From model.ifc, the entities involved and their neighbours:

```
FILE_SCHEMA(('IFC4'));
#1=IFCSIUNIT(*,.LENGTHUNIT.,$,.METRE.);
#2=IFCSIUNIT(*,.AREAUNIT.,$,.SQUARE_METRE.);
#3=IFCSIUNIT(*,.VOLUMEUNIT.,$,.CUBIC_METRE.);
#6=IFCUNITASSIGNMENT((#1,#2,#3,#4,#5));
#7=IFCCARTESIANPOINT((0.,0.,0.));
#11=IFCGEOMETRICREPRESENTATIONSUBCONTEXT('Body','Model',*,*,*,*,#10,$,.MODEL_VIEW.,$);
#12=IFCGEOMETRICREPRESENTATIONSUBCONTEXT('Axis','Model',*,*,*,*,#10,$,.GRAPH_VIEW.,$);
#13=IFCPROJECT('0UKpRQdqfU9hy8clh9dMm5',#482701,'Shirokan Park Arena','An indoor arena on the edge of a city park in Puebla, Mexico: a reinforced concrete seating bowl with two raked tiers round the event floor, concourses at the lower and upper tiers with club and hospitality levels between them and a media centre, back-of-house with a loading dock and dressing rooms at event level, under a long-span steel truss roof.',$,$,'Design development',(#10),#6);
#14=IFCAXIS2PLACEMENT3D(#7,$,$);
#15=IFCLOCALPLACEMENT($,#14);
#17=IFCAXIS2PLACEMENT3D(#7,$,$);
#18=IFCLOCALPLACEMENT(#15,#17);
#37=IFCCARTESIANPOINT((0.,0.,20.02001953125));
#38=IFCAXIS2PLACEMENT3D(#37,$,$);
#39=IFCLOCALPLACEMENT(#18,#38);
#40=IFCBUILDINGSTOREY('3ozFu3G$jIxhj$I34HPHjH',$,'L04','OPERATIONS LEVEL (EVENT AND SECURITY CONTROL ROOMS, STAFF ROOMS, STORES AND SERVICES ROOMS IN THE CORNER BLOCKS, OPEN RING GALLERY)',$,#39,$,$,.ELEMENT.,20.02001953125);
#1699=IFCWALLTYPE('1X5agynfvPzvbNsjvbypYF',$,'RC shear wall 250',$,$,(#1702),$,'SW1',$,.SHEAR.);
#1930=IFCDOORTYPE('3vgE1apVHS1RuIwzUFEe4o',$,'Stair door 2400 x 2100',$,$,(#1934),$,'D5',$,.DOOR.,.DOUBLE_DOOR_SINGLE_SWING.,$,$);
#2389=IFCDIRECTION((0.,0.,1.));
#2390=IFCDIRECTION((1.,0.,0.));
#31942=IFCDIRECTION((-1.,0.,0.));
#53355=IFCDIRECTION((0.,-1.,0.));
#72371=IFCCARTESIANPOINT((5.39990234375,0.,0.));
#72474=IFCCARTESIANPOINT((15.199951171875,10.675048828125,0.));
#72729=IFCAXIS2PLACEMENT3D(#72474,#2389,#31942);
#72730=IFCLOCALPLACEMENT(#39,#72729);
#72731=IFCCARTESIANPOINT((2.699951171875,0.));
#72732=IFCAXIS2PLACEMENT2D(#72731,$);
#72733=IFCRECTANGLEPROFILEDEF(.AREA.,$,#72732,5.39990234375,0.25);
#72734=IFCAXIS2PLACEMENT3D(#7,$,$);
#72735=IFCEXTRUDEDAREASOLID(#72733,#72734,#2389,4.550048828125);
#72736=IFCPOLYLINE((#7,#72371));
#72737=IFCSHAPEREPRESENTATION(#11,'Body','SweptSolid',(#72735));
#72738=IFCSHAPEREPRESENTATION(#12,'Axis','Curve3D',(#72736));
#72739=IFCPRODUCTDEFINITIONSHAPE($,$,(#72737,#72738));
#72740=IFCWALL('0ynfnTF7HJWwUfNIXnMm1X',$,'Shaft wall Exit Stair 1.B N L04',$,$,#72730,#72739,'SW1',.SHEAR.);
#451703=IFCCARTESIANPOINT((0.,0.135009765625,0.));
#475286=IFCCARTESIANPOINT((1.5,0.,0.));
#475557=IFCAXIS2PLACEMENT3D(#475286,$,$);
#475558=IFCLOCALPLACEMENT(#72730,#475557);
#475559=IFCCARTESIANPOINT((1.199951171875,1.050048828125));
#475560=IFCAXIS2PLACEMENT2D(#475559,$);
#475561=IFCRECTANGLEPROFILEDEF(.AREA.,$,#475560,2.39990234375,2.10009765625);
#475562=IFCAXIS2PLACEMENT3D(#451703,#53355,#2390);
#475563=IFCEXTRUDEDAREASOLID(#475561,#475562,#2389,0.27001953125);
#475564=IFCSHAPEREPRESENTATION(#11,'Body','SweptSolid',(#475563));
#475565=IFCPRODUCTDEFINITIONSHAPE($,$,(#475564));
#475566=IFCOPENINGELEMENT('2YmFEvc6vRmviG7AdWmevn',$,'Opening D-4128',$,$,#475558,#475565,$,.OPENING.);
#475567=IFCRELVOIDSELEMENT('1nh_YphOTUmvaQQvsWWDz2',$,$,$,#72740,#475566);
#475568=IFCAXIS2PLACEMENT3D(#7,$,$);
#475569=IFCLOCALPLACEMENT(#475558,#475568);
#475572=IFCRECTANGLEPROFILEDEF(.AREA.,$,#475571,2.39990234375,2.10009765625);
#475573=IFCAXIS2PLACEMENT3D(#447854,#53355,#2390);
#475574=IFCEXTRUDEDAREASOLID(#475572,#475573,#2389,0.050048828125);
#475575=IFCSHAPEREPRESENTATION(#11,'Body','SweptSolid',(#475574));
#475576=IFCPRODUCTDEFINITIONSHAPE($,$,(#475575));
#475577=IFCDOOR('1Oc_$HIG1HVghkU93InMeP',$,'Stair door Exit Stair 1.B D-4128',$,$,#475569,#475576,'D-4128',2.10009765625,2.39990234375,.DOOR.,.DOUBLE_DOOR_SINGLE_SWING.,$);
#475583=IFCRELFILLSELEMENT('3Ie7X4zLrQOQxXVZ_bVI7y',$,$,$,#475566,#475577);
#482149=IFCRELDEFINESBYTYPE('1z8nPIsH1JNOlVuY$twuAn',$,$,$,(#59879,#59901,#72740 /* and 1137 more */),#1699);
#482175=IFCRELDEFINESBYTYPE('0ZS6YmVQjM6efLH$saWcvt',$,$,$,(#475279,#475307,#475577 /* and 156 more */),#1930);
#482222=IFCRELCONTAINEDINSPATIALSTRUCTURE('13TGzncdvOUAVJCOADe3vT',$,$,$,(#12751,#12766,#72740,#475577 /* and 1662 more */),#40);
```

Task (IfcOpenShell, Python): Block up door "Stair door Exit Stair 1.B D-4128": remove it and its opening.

```python
import ifcopenshell
import ifcopenshell.api.feature
import ifcopenshell.api.root
import ifcopenshell.geom
import ifcopenshell.util.shape

model = ifcopenshell.open("model.ifc")
settings = ifcopenshell.geom.settings()


def volume(element):
    """Net volume in cubic metres, openings subtracted."""
    shape = ifcopenshell.geom.create_shape(settings, element)
    return ifcopenshell.util.shape.get_volume(shape.geometry)


door = model.by_guid("1Oc_$HIG1HVghkU93InMeP")
opening = door.FillsVoids[0].RelatingOpeningElement
wall = opening.VoidsElements[0].RelatingBuildingElement
before = volume(wall)

ifcopenshell.api.root.remove_product(model, product=door)
ifcopenshell.api.feature.remove_feature(model, feature=opening)

after = volume(wall)

print(f"wall volume {before:.3f} -> {after:.3f} m3")

model.write("model-out.ifc")
```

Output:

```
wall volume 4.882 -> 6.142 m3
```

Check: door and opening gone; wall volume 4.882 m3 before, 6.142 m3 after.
